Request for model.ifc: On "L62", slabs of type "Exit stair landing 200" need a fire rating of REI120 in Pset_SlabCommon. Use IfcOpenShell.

First a look at what the model holds.

```python
import ifcopenshell
import ifcopenshell.util.element

model = ifcopenshell.open("model.ifc")
print(model.schema)
storey = next(s for s in model.by_type("IfcBuildingStorey") if s.Name == "L62")
slabs = [e for e in ifcopenshell.util.element.get_decomposition(storey) if e.is_a("IfcSlab")]
seen = {}
for e in slabs:
    element_type = ifcopenshell.util.element.get_type(e)
    key = (element_type.Name if element_type != e and element_type else None, ifcopenshell.util.element.get_pset(e, "Pset_SlabCommon", "FireRating"))
    seen[key] = seen.get(key, 0) + 1
for (name, value), count in sorted(seen.items(), key=str):
    print(count, "x", name, "|", value)
```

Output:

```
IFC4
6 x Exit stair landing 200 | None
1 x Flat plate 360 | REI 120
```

```python
import ifcopenshell
import ifcopenshell.api.pset
import ifcopenshell.util.element

model = ifcopenshell.open("model.ifc")

storey = next(s for s in model.by_type("IfcBuildingStorey") if s.Name == "L62")
slabs = [e for e in ifcopenshell.util.element.get_decomposition(storey) if e.is_a("IfcSlab")]

count = 0
for e in slabs:
    element_type = ifcopenshell.util.element.get_type(e)
    if element_type in (None, e) or element_type.Name != "Exit stair landing 200":
        continue
    found = ifcopenshell.util.element.get_pset(e, "Pset_SlabCommon", should_inherit=False)
    if found:
        pset = model.by_id(found["id"])
        if len(ifcopenshell.util.element.get_elements_by_pset(pset)) > 1:
            pset = ifcopenshell.api.pset.unshare_pset(model, products=[e], pset=pset)[0]
    else:
        pset = ifcopenshell.api.pset.add_pset(model, product=e, name="Pset_SlabCommon")
    ifcopenshell.api.pset.edit_pset(model, pset=pset, properties={"FireRating": "REI120"})
    count += 1

print(count, "slabs updated")

model.write("model_edited.ifc")
```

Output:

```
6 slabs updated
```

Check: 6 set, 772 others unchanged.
